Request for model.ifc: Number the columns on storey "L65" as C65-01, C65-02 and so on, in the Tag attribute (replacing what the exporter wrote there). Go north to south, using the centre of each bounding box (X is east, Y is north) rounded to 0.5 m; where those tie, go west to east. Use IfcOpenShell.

First a look at what the model holds.

```python
import ifcopenshell
import ifcopenshell.util.element
import ifcopenshell.util.placement

model = ifcopenshell.open("model.ifc")
print(model.schema)
storey = next(s for s in model.by_type("IfcBuildingStorey") if s.Name == "L65")
columns = [e for e in ifcopenshell.util.element.get_decomposition(storey) if e.is_a("IfcColumn")]
for e in sorted(columns, key=lambda e: e.id()):
    origin = ifcopenshell.util.placement.get_local_placement(e.ObjectPlacement)[:3, 3]
    print(e.id(), e.Tag, e.Name, origin.round(2) + 0.0, sep=" | ")
```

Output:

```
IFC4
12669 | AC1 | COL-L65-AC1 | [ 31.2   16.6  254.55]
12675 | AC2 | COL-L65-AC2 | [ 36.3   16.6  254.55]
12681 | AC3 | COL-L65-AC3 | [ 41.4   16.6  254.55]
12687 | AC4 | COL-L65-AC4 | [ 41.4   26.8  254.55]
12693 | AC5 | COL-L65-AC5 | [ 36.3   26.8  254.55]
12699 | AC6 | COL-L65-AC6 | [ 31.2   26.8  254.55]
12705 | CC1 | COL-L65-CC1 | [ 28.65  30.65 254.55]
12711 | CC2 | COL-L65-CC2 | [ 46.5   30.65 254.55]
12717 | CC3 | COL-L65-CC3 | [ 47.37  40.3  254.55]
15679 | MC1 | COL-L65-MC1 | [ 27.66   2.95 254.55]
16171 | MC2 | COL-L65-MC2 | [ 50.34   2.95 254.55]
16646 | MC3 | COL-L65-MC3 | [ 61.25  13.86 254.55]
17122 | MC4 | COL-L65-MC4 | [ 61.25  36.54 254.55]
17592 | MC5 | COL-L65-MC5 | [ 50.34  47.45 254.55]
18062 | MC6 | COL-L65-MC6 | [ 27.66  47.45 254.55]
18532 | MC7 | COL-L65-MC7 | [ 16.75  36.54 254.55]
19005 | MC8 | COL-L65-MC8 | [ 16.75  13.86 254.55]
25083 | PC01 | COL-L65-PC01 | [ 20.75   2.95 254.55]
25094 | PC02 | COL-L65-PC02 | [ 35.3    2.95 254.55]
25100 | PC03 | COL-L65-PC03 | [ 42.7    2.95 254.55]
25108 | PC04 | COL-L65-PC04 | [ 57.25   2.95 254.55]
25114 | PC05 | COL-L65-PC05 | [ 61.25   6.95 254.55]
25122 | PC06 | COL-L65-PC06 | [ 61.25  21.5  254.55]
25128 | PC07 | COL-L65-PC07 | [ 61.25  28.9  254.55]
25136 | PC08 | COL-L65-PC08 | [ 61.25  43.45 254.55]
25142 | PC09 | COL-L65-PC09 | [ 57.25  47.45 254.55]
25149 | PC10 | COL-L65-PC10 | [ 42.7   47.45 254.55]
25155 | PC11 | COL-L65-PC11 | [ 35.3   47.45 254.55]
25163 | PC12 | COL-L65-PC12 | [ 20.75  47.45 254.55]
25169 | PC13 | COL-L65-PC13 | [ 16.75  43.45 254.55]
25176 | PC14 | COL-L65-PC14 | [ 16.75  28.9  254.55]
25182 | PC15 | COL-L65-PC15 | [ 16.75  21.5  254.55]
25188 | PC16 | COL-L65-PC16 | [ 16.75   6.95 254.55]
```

```python
import ifcopenshell
import ifcopenshell.geom
import ifcopenshell.util.element
import ifcopenshell.util.shape

model = ifcopenshell.open("model.ifc")
settings = ifcopenshell.geom.settings()
settings.set("use-world-coords", True)


def centre(element):
    shape = ifcopenshell.geom.create_shape(settings, element)
    return ifcopenshell.util.shape.get_bbox_centroid(shape.geometry)


storey = next(s for s in model.by_type("IfcBuildingStorey") if s.Name == "L65")
columns = [e for e in ifcopenshell.util.element.get_decomposition(storey) if e.is_a("IfcColumn")]

# Insertion points can sit at a corner or the storey origin, so sort by the geometry (in metres).
centres = {e: centre(e) for e in columns}
columns.sort(key=lambda e: (-round(centres[e][1] / 0.5), centres[e][0]))

for i, e in enumerate(columns, start=1):
    number = f"C65-{i:02d}"
    e.Tag = number
    print(e.id(), number)

model.write("model_v2.ifc")
```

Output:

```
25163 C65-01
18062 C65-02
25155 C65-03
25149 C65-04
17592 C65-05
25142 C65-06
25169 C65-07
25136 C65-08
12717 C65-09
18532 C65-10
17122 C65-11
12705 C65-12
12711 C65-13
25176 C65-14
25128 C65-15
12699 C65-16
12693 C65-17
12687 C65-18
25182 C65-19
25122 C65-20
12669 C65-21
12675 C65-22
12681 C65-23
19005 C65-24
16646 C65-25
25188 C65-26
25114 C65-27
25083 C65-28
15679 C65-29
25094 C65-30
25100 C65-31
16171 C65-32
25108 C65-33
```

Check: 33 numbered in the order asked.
